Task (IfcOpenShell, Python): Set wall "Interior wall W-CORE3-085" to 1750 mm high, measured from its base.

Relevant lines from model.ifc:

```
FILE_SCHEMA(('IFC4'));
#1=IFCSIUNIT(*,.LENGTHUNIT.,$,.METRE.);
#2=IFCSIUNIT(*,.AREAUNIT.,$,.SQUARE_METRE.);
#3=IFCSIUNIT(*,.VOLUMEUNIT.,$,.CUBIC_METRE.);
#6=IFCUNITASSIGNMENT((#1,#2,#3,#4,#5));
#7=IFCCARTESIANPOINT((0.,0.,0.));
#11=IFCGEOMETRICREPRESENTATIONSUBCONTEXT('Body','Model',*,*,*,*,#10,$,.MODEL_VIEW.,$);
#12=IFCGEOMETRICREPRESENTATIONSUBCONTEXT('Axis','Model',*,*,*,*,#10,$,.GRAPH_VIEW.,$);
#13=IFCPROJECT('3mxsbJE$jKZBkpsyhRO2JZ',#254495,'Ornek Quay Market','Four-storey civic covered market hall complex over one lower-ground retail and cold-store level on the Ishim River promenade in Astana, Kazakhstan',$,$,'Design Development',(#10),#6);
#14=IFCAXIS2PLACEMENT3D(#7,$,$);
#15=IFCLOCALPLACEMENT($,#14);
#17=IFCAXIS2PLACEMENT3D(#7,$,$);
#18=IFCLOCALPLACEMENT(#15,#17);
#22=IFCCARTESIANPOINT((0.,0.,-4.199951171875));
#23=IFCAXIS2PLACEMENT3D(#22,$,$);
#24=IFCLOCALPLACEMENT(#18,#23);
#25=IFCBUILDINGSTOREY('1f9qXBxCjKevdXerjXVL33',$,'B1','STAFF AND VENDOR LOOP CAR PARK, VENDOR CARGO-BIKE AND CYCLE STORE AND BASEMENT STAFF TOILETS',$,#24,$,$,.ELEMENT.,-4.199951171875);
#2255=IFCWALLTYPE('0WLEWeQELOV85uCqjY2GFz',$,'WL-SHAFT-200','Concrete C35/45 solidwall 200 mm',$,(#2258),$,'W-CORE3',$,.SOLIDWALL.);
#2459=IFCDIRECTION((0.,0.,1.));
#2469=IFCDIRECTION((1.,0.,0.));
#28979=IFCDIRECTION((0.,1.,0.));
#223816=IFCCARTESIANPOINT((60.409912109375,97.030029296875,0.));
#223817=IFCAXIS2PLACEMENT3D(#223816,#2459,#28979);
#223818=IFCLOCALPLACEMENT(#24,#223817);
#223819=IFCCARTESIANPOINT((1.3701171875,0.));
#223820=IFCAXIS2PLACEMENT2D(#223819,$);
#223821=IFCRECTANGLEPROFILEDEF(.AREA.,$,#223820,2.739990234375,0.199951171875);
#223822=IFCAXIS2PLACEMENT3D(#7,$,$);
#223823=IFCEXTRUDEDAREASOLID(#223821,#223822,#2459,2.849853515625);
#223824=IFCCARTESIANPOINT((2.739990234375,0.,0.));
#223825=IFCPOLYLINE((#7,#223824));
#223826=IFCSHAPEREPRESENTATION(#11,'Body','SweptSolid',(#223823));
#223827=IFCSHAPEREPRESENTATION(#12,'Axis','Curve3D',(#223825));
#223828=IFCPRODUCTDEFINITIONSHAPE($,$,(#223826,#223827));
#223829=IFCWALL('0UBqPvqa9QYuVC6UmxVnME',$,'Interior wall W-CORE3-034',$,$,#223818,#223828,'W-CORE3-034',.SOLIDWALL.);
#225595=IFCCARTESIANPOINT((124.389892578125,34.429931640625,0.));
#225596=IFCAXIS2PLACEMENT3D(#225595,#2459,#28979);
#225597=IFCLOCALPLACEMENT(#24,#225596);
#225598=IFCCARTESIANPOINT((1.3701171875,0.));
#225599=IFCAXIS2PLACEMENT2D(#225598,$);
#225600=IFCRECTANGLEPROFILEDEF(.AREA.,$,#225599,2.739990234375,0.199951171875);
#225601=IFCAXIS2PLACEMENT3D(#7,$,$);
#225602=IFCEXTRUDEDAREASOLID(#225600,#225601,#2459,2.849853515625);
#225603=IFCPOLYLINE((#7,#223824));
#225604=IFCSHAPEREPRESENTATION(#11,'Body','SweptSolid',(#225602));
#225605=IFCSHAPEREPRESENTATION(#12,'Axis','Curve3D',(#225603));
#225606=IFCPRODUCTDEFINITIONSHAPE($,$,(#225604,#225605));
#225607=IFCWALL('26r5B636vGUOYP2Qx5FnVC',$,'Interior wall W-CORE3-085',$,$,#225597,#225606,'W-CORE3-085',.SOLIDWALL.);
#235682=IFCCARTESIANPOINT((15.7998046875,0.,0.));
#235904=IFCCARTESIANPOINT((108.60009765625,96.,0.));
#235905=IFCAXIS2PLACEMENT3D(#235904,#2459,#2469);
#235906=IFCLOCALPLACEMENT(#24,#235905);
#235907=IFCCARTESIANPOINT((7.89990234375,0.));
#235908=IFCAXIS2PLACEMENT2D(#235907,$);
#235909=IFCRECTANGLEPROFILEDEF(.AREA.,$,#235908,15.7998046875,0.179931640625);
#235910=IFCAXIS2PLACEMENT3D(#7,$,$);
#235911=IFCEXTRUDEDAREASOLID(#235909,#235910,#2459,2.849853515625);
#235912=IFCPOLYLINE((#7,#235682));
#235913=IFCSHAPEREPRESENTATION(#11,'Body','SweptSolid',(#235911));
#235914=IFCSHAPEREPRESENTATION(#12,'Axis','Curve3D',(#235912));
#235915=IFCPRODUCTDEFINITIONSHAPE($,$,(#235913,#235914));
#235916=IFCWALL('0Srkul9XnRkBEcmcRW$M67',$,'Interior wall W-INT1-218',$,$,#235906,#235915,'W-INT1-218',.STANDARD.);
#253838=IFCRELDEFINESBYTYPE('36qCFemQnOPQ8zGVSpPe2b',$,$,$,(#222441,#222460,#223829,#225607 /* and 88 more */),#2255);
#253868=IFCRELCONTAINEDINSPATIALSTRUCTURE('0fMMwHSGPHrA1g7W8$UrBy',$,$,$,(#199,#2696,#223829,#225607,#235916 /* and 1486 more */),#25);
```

```python
import ifcopenshell
import ifcopenshell.geom
import ifcopenshell.util.representation
import ifcopenshell.util.shape
import ifcopenshell.util.unit

model = ifcopenshell.open("model.ifc")
unit_scale = ifcopenshell.util.unit.calculate_unit_scale(model)
settings = ifcopenshell.geom.settings()


def volume(element):
    """Net volume in cubic metres, openings subtracted."""
    shape = ifcopenshell.geom.create_shape(settings, element)
    return ifcopenshell.util.shape.get_volume(shape.geometry)


wall = model.by_guid("26r5B636vGUOYP2Qx5FnVC")
before = volume(wall)

body = ifcopenshell.util.representation.get_representation(wall, "Model", "Body")
solid = body.Items[0]
old_height = solid.Depth
solid.Depth = 1.75 / unit_scale
after = volume(wall)

print(f"height {old_height:g} -> {solid.Depth:g}, volume {before:.3f} -> {after:.3f} m3")

model.write("model_v2.ifc")
```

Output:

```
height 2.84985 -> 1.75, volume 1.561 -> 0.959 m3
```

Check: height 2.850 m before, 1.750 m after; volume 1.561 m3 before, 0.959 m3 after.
